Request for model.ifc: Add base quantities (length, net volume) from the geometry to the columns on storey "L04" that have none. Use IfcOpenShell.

First a look at what the model holds.

```python
import ifcopenshell
import ifcopenshell.util.element
import ifcopenshell.util.unit

model = ifcopenshell.open("model.ifc")
print(model.schema)
for unit_type in ("LENGTHUNIT", "AREAUNIT", "VOLUMEUNIT"):
    print(unit_type, ifcopenshell.util.unit.calculate_unit_scale(model, unit_type))
storey = next(s for s in model.by_type("IfcBuildingStorey") if s.Name == "L04")
columns = [e for e in ifcopenshell.util.element.get_decomposition(storey) if e.is_a("IfcColumn")]
for e in sorted(columns, key=lambda e: e.id()):
    print(e.id(), e.is_a(), e.Name, list(ifcopenshell.util.element.get_psets(e, qtos_only=True)), sep=" | ")
```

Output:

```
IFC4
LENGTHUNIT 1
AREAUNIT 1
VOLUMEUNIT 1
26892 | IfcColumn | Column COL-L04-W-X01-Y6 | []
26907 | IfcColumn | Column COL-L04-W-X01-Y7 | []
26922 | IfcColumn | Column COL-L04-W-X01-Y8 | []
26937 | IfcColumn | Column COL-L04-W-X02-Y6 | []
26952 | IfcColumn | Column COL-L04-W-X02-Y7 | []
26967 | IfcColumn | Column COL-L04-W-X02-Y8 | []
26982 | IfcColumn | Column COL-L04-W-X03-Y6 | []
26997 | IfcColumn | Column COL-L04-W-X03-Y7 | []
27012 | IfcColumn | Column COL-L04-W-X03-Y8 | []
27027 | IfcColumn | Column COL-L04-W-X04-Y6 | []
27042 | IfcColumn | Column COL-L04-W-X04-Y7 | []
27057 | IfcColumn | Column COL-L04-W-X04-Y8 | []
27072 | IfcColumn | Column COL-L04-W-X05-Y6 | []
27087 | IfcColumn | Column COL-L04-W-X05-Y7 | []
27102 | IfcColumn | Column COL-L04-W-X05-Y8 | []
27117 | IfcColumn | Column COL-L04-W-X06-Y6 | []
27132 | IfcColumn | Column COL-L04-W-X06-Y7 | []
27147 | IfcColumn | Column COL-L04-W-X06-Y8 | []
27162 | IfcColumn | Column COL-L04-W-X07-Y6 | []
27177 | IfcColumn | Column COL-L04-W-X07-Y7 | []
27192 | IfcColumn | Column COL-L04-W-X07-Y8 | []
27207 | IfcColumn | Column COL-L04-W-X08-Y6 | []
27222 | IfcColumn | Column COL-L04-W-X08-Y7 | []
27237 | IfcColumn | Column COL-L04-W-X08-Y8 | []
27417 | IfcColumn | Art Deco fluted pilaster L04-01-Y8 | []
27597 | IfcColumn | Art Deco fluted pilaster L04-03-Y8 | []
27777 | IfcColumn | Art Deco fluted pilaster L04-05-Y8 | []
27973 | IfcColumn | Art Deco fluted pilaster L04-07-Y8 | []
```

```python
import ifcopenshell
import ifcopenshell.api.pset
import ifcopenshell.geom
import ifcopenshell.util.element
import ifcopenshell.util.shape
import ifcopenshell.util.unit

model = ifcopenshell.open("model.ifc")
unit_scale = ifcopenshell.util.unit.calculate_unit_scale(model)
volume_scale = ifcopenshell.util.unit.calculate_unit_scale(model, "VOLUMEUNIT")
settings = ifcopenshell.geom.settings()

storey = next(s for s in model.by_type("IfcBuildingStorey") if s.Name == "L04")
columns = [e for e in ifcopenshell.util.element.get_decomposition(storey) if e.is_a("IfcColumn")]

for e in sorted(columns, key=lambda e: e.id()):
    if ifcopenshell.util.element.get_psets(e, qtos_only=True, should_inherit=False):
        continue
    # Geometry comes back in metres, in the element's own axes.
    shape = ifcopenshell.geom.create_shape(settings, e)
    values = {
        "Length": ifcopenshell.util.shape.get_z(shape.geometry) / unit_scale,
        "NetVolume": ifcopenshell.util.shape.get_volume(shape.geometry) / volume_scale,
    }
    qto = ifcopenshell.api.pset.add_qto(model, product=e, name="Qto_ColumnBaseQuantities")
    ifcopenshell.api.pset.edit_qto(model, qto=qto, properties=values)
    print(e.id(), {k: round(v, 3) for k, v in values.items()})

model.write("model_edited.ifc")
```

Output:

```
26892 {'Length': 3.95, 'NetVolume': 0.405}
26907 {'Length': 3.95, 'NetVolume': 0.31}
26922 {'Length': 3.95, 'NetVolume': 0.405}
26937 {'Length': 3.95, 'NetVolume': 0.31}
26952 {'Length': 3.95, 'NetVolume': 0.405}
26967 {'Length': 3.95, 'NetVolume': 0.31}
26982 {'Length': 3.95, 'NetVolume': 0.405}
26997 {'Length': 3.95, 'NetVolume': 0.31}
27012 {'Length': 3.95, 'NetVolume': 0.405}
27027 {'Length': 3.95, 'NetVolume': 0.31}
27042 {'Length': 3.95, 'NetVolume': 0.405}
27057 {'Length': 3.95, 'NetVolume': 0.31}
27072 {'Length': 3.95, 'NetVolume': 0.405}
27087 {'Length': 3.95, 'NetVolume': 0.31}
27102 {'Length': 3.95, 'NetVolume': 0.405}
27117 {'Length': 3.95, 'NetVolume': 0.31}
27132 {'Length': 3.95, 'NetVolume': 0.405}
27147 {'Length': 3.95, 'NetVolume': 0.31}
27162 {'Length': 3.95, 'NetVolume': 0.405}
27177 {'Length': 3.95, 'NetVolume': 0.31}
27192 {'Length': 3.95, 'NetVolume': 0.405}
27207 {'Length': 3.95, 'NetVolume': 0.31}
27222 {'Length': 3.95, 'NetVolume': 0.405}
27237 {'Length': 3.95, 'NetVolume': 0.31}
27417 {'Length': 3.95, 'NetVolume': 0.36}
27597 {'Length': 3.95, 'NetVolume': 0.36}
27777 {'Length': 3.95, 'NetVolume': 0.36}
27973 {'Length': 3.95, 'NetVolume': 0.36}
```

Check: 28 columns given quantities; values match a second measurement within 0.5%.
